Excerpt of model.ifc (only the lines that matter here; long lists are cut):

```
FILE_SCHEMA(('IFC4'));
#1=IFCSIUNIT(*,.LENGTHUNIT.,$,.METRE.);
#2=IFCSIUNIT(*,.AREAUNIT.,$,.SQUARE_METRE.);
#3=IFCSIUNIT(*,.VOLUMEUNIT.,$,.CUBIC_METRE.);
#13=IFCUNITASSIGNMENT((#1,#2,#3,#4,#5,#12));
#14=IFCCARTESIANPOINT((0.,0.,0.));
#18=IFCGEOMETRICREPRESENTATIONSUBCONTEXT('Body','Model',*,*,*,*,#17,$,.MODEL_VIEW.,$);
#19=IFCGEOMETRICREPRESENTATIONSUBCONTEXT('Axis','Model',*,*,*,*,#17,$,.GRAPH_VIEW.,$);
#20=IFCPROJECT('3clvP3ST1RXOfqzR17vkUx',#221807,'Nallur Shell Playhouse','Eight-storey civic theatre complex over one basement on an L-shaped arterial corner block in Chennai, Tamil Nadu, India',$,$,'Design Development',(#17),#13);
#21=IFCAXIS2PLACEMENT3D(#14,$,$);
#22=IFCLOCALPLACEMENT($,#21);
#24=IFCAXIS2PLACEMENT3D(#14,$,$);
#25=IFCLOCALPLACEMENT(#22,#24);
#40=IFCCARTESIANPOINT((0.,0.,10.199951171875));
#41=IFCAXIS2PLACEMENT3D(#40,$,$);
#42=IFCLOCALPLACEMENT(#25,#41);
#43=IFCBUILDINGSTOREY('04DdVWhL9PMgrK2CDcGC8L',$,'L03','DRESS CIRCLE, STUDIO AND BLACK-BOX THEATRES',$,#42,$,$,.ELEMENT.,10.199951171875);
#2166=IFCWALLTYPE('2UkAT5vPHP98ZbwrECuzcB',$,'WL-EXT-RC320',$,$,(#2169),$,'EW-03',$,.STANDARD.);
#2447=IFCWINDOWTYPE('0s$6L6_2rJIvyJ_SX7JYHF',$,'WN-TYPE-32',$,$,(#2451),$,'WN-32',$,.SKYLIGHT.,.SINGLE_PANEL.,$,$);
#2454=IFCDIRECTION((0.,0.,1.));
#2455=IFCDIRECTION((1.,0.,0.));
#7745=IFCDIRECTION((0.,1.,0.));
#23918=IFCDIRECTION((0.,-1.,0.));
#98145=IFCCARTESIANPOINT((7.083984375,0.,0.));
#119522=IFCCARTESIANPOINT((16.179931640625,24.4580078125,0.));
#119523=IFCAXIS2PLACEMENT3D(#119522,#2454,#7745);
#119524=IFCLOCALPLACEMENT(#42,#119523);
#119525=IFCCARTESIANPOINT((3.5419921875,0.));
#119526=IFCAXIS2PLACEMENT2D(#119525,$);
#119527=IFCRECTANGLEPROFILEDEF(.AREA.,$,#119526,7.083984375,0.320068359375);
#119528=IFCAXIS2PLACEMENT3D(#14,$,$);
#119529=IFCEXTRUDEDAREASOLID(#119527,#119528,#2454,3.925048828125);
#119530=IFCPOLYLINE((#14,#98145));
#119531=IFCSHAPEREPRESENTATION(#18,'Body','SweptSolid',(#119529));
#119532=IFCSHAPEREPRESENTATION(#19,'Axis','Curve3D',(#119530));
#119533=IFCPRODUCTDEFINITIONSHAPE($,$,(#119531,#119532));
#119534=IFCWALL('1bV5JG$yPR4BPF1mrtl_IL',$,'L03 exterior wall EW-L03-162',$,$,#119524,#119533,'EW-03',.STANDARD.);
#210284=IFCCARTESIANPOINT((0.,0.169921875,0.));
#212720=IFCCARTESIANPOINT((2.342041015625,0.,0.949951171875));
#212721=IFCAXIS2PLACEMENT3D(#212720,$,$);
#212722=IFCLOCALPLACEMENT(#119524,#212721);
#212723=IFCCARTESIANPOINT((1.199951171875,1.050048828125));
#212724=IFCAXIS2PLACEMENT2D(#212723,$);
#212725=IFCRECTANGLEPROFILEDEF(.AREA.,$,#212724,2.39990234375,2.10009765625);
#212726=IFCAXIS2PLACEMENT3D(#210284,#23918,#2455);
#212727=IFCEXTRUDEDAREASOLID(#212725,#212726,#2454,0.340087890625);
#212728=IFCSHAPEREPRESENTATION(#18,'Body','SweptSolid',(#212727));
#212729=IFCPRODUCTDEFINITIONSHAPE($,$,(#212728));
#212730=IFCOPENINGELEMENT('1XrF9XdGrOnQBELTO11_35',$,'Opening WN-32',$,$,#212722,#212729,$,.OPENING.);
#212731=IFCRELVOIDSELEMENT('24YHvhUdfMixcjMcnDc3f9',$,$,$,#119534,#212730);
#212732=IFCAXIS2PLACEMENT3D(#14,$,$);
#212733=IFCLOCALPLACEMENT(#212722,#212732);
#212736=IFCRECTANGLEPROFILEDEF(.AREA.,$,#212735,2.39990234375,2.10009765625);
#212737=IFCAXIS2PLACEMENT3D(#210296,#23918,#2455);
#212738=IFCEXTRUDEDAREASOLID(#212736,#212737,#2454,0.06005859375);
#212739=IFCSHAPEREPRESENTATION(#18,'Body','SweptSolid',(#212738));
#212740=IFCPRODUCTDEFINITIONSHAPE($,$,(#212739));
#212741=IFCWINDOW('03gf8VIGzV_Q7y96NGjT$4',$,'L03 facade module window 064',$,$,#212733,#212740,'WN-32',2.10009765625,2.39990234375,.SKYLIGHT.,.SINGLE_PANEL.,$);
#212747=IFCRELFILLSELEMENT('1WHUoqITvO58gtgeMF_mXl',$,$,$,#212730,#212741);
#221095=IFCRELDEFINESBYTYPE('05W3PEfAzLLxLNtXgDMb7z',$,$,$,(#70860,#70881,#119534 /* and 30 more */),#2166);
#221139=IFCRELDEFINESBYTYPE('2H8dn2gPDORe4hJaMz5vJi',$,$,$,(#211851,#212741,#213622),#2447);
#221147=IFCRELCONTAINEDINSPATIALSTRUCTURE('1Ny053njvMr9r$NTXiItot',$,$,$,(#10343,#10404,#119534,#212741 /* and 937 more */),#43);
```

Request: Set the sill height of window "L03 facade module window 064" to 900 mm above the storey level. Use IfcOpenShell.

```python
import numpy as np
import ifcopenshell
import ifcopenshell.api.geometry
import ifcopenshell.geom
import ifcopenshell.util.element
import ifcopenshell.util.placement
import ifcopenshell.util.shape
import ifcopenshell.util.unit

model = ifcopenshell.open("model.ifc")
unit_scale = ifcopenshell.util.unit.calculate_unit_scale(model)

window = model.by_guid("03gf8VIGzV_Q7y96NGjT$4")
opening = window.FillsVoids[0].RelatingOpeningElement
storey = ifcopenshell.util.element.get_container(window, ifc_class="IfcBuildingStorey")
level = ifcopenshell.util.placement.get_local_placement(storey.ObjectPlacement)[2, 3]

# The opening's origin need not be at the sill, so measure its lowest point.
shape = ifcopenshell.geom.create_shape(ifcopenshell.geom.settings(), opening)
bottom = ifcopenshell.util.shape.get_shape_bottom_elevation(shape, shape.geometry) / unit_scale
dz = level + 0.9 / unit_scale - bottom

shift = np.array([0.0, 0.0, dz])
# The window is placed relative to its opening, so it follows when the opening moves.
matrix = ifcopenshell.util.placement.get_local_placement(opening.ObjectPlacement)
matrix[:3, 3] += shift
ifcopenshell.api.geometry.edit_object_placement(
    model, product=opening, matrix=matrix, is_si=False, should_transform_children=True
)

print(f"moved by {dz * unit_scale:+.3f} m")

model.write("model-out.ifc")
```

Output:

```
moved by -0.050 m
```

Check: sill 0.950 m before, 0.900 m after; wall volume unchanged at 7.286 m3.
